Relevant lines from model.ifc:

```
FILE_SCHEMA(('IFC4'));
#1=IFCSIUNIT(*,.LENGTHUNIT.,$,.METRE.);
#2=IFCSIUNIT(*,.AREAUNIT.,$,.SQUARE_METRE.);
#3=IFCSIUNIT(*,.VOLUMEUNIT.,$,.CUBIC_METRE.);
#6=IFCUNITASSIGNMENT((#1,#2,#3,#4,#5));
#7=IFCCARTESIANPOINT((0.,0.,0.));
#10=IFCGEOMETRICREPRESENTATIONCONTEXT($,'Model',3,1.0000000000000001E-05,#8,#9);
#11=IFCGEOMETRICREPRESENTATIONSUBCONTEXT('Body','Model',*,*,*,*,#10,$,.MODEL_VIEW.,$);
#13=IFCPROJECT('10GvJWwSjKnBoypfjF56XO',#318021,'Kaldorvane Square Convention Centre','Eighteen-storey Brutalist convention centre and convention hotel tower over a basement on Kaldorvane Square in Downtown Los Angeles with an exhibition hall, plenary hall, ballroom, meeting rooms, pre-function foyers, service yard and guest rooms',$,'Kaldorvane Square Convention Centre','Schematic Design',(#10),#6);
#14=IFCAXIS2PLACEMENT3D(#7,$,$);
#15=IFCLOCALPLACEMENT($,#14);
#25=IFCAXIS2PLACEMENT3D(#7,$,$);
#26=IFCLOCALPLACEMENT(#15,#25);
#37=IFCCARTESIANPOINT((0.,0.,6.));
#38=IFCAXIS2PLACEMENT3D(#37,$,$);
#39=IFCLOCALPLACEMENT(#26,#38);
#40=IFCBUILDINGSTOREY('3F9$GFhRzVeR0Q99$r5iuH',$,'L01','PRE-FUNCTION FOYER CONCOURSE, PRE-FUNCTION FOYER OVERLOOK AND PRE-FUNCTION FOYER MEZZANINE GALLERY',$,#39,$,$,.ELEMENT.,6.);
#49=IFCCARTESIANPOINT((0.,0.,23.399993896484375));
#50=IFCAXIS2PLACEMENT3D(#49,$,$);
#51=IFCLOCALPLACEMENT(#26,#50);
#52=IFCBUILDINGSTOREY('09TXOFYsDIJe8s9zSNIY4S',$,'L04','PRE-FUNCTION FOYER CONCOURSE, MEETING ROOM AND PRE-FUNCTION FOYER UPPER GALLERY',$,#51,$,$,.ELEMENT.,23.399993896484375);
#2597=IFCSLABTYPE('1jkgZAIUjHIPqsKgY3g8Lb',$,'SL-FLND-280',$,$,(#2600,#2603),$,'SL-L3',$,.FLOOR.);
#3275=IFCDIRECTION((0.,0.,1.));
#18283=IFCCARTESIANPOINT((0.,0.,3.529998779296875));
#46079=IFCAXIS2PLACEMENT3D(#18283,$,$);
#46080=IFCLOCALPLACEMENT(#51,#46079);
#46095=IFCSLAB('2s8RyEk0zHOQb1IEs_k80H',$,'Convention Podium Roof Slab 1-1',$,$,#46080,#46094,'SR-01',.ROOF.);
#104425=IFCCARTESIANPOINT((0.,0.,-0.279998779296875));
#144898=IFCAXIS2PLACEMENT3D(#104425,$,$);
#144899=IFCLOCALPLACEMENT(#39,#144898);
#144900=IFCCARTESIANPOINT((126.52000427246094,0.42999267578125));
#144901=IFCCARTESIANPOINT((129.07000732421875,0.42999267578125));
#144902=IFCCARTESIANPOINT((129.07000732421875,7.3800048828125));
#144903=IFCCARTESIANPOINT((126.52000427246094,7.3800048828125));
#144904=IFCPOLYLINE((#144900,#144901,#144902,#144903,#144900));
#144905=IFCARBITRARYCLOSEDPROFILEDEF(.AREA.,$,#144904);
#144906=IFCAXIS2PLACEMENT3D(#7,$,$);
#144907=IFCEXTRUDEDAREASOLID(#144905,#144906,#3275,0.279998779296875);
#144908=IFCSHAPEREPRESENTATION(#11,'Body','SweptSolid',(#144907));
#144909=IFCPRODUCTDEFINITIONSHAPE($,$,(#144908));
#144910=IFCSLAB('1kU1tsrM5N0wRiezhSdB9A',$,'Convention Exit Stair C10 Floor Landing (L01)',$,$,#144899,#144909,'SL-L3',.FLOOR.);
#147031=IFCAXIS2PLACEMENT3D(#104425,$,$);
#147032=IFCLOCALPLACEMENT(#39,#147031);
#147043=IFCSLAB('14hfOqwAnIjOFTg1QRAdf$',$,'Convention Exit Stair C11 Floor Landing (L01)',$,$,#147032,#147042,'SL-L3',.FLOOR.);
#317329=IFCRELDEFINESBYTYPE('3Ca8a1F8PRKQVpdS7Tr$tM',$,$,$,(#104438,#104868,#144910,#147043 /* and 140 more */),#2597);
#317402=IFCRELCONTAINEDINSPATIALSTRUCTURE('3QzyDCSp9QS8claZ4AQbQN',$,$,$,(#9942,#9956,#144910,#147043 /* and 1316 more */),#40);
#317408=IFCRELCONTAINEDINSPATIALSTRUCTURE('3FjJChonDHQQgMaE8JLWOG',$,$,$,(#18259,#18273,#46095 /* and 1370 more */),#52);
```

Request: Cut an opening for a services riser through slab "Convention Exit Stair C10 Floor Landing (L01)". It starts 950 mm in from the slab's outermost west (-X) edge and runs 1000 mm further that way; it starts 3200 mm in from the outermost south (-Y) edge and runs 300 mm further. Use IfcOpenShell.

```python
import numpy as np
import ifcopenshell
import ifcopenshell.api.feature
import ifcopenshell.api.geometry
import ifcopenshell.api.root
import ifcopenshell.geom
import ifcopenshell.util.placement
import ifcopenshell.util.representation
import ifcopenshell.util.shape
import ifcopenshell.util.unit

model = ifcopenshell.open("model.ifc")
unit_scale = ifcopenshell.util.unit.calculate_unit_scale(model)
settings = ifcopenshell.geom.settings()


def volume(element):
    """Net volume in cubic metres, openings subtracted."""
    shape = ifcopenshell.geom.create_shape(settings, element)
    return ifcopenshell.util.shape.get_volume(shape.geometry)


slab = model.by_guid("1kU1tsrM5N0wRiezhSdB9A")
before = volume(slab)

# Extent in the slab's own axes, in metres. The edges named are its -X and -Y sides.
slab_shape = ifcopenshell.geom.create_shape(settings, slab)
vertices = ifcopenshell.util.shape.get_vertices(slab_shape.geometry)
x_min, y_min, bottom = vertices.min(axis=0)
top = vertices[:, 2].max()

opening = ifcopenshell.api.root.create_entity(model, ifc_class="IfcOpeningElement", name="Services riser opening", predefined_type="OPENING")
context = ifcopenshell.util.representation.get_context(model, "Model", "Body", "MODEL_VIEW")
width, depth = 1, 0.3
outline = [(0.0, 0.0), (width, 0.0), (width, depth), (0.0, depth), (0.0, 0.0)]
# Overshoot both faces by 50 mm so the cut is clean.
shape = ifcopenshell.api.geometry.add_slab_representation(
    model, context=context, depth=top - bottom + 0.1, polyline=outline
)
ifcopenshell.api.geometry.assign_representation(model, product=opening, representation=shape)

matrix = ifcopenshell.util.placement.get_local_placement(slab.ObjectPlacement)
matrix[:, 3] = matrix @ np.append(np.array([x_min + 0.95, y_min + 3.2, bottom - 0.05]) / unit_scale, 1.0)
ifcopenshell.api.geometry.edit_object_placement(model, product=opening, matrix=matrix, is_si=False)
ifcopenshell.api.feature.add_feature(model, feature=opening, element=slab)

after = volume(slab)

print(f"slab volume {before:.3f} -> {after:.3f} m3")

model.write("model_updated.ifc")
```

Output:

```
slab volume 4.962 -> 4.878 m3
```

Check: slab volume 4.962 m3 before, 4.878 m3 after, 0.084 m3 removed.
